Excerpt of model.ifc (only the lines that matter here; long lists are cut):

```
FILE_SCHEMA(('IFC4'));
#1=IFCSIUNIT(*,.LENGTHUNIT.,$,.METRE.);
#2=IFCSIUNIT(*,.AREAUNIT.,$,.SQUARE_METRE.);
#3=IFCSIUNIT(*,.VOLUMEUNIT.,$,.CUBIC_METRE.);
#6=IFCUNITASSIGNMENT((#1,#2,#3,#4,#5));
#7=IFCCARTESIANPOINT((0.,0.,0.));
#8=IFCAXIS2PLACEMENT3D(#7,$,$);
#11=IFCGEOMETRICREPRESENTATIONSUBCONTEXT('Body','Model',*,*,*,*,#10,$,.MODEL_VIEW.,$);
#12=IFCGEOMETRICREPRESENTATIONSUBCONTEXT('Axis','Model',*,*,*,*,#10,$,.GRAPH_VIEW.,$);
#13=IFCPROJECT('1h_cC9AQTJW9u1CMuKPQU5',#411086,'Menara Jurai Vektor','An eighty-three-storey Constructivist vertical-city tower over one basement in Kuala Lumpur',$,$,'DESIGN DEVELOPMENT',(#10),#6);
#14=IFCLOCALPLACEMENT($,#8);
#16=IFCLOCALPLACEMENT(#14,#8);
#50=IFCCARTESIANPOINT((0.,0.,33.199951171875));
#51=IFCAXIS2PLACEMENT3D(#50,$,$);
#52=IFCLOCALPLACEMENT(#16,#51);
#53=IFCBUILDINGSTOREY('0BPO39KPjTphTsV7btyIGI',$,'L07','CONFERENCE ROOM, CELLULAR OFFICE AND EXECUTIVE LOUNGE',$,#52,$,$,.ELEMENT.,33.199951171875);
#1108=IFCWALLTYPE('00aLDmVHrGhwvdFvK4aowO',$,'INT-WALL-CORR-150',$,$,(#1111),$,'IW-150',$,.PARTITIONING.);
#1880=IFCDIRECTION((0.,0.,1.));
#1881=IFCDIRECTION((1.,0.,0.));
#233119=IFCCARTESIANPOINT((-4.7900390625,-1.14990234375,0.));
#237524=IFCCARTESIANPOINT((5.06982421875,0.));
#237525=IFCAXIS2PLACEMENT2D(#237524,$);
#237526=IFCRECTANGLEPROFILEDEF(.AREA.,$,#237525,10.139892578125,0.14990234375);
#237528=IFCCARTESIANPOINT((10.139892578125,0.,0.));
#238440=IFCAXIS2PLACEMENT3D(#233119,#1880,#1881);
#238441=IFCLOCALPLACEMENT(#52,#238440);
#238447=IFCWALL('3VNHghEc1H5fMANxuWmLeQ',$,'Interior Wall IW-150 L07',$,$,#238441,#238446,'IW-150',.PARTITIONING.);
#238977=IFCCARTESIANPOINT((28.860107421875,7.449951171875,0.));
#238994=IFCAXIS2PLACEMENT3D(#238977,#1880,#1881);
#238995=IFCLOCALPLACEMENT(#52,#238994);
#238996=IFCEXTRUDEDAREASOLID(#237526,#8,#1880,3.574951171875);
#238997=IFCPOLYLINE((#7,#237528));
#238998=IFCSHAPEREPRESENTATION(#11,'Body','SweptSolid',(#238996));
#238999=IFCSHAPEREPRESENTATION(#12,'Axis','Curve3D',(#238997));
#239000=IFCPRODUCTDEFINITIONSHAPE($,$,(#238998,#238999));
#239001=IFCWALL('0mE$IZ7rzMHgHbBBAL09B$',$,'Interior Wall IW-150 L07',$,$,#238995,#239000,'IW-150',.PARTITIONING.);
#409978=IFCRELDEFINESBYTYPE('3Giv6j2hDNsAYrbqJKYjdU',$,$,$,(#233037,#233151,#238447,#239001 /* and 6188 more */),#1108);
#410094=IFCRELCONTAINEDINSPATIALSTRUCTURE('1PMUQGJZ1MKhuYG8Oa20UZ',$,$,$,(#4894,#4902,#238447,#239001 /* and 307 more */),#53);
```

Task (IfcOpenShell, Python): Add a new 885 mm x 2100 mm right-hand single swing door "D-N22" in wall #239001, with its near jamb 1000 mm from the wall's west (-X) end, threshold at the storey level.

```python
import numpy as np
import ifcopenshell
import ifcopenshell.api.feature
import ifcopenshell.api.geometry
import ifcopenshell.api.root
import ifcopenshell.api.spatial
import ifcopenshell.geom
import ifcopenshell.util.element
import ifcopenshell.util.placement
import ifcopenshell.util.representation
import ifcopenshell.util.shape
import ifcopenshell.util.unit

model = ifcopenshell.open("model.ifc")
unit_scale = ifcopenshell.util.unit.calculate_unit_scale(model)
settings = ifcopenshell.geom.settings()


def volume(element):
    """Net volume in cubic metres, openings subtracted."""
    shape = ifcopenshell.geom.create_shape(settings, element)
    return ifcopenshell.util.shape.get_volume(shape.geometry)


wall = model.by_guid("0mE$IZ7rzMHgHbBBAL09B$")
storey = ifcopenshell.util.element.get_container(wall, ifc_class="IfcBuildingStorey")
context = ifcopenshell.util.representation.get_context(model, "Model", "Body", "MODEL_VIEW")
before = volume(wall)

width, height, from_end, sill = 0.885, 2.1, 1, 0.0  # metres

# The wall runs along its own X axis, and the end named is its -X end.
wall_shape = ifcopenshell.geom.create_shape(settings, wall)
x, y, z = ifcopenshell.util.shape.get_vertices(wall_shape.geometry).T
start = x.min() + from_end
face, thickness = float(y.min()), float(y.max() - y.min())
wall_matrix = ifcopenshell.util.placement.get_local_placement(wall.ObjectPlacement)
level = ifcopenshell.util.placement.get_local_placement(storey.ObjectPlacement)[2, 3]


def in_wall(x, y):
    """Placement at x, y metres in the wall's axes, at sill height."""
    matrix = wall_matrix.copy()
    matrix[:, 3] = wall_matrix @ np.array([x / unit_scale, y / unit_scale, 0.0, 1.0])
    matrix[2, 3] = level + sill / unit_scale
    return matrix


# Opening: a box that overshoots both wall faces by 50 mm.
opening = ifcopenshell.api.root.create_entity(model, ifc_class="IfcOpeningElement", predefined_type="OPENING")
box = ifcopenshell.api.geometry.add_wall_representation(
    model, context=context, length=width, height=height, thickness=thickness + 0.1
)
ifcopenshell.api.geometry.assign_representation(model, product=opening, representation=box)
ifcopenshell.api.geometry.edit_object_placement(model, product=opening, matrix=in_wall(start, face - 0.05), is_si=False)
ifcopenshell.api.feature.add_feature(model, feature=opening, element=wall)

door = ifcopenshell.api.root.create_entity(model, ifc_class="IfcDoor", name="D-N22", predefined_type="DOOR")
door.OverallWidth, door.OverallHeight = width / unit_scale, height / unit_scale
door.OperationType = "SINGLE_SWING_RIGHT"
body = ifcopenshell.api.geometry.add_door_representation(
    model,
    context=context,
    overall_width=door.OverallWidth,
    overall_height=door.OverallHeight,
    operation_type="SINGLE_SWING_RIGHT",
    lining_properties={"LiningDepth": thickness / unit_scale, "ThresholdDepth": thickness / unit_scale},
)
ifcopenshell.api.geometry.assign_representation(model, product=door, representation=body)
ifcopenshell.api.spatial.assign_container(model, products=[door], relating_structure=storey)
ifcopenshell.api.feature.add_filling(model, opening=opening, element=door)

# The lining spans the wall, so the door starts at the wall face.
ifcopenshell.api.geometry.edit_object_placement(model, product=door, matrix=in_wall(start, face), is_si=False)

after = volume(wall)

print(f"wall volume {before:.3f} -> {after:.3f} m3")

model.write("model_rev.ifc")
```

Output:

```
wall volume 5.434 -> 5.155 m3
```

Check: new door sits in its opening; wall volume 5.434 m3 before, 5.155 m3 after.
